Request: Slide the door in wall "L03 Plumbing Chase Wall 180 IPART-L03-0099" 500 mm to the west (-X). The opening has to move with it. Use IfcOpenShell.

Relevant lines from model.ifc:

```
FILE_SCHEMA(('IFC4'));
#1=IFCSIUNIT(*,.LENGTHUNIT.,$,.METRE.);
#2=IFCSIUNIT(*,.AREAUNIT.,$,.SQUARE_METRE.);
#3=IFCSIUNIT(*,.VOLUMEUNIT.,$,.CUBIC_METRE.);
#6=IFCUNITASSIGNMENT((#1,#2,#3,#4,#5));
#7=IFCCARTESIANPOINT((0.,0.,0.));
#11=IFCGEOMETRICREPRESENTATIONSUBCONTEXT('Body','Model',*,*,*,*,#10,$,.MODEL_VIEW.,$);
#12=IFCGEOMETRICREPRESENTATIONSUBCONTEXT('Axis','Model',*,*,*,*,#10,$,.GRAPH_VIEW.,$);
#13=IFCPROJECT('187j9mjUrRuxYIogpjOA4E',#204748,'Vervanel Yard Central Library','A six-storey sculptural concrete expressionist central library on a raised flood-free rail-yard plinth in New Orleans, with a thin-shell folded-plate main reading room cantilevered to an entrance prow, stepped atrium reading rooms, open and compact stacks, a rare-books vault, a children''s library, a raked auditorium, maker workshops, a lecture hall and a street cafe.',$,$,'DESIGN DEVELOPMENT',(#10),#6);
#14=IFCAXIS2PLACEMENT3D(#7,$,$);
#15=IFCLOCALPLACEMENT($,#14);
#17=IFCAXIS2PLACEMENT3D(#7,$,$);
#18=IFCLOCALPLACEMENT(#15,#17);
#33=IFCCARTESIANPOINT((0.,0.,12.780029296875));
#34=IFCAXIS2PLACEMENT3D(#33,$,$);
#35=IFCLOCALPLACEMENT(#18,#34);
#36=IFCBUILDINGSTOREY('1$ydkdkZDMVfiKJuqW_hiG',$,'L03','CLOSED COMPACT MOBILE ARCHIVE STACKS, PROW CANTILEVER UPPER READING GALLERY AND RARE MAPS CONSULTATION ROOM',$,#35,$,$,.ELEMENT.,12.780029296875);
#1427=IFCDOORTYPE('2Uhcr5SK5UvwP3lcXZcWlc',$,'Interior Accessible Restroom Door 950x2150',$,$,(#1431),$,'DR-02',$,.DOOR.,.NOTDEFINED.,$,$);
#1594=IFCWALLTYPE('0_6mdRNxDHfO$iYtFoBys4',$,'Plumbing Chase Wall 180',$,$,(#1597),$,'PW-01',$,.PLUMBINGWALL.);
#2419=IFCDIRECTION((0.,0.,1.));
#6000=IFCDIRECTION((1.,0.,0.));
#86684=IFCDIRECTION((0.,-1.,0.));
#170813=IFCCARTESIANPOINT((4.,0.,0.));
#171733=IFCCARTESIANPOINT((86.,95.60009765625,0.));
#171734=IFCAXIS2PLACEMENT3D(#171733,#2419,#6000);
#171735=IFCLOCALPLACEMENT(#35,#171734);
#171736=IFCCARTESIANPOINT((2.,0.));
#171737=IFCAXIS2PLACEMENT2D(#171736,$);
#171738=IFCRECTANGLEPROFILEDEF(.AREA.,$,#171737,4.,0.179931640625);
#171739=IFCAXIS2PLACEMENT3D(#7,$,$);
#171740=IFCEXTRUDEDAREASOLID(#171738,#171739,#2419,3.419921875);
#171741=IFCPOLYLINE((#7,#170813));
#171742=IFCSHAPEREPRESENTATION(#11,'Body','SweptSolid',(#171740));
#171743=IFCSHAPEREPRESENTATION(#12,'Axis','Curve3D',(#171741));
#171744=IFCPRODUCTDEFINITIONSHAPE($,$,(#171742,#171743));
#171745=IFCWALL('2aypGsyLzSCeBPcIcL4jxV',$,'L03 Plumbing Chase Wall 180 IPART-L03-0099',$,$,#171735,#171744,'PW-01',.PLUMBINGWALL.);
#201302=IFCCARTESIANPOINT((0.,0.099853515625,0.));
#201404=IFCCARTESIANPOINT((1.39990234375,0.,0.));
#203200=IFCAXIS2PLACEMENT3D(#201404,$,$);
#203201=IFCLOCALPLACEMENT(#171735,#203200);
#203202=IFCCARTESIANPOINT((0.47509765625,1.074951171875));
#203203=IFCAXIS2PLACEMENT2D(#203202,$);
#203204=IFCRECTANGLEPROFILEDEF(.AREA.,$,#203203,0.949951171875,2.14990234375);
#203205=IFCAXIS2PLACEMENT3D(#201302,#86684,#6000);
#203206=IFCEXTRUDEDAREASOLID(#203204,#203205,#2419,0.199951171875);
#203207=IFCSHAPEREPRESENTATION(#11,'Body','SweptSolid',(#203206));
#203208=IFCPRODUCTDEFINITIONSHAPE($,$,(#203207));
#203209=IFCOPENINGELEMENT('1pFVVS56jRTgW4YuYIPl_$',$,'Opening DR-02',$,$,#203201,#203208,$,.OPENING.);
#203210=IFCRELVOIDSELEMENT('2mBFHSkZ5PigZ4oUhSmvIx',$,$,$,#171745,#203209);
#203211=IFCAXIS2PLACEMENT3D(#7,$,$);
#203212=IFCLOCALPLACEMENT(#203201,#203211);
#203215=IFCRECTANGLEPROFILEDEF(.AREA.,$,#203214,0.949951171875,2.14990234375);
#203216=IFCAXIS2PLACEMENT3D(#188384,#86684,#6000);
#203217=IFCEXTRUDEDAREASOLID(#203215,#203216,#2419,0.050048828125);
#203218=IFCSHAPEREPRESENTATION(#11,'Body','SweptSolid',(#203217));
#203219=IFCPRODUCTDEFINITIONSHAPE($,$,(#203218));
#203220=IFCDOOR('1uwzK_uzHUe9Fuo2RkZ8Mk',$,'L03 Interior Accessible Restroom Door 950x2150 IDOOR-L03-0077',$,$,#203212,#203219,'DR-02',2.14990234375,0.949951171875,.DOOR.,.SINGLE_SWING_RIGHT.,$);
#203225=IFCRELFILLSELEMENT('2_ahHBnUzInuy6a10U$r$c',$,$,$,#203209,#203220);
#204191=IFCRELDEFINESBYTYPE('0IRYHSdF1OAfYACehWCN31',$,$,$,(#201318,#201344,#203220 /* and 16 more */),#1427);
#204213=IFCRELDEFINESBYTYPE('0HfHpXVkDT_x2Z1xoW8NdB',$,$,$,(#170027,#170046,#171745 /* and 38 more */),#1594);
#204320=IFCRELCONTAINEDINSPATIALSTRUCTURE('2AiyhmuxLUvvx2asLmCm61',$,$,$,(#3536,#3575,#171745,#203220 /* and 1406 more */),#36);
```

```python
import ifcopenshell
import ifcopenshell.api.geometry
import ifcopenshell.util.placement

model = ifcopenshell.open("model.ifc")

door = model.by_guid("1uwzK_uzHUe9Fuo2RkZ8Mk")
opening = door.FillsVoids[0].RelatingOpeningElement
wall = opening.VoidsElements[0].RelatingBuildingElement

wall_matrix = ifcopenshell.util.placement.get_local_placement(wall.ObjectPlacement)
shift = wall_matrix[:3, 0] * -0.5
before = ifcopenshell.util.placement.get_local_placement(door.ObjectPlacement)[:3, 3].copy()

# The door is placed relative to its opening, so it follows when the opening moves.
matrix = ifcopenshell.util.placement.get_local_placement(opening.ObjectPlacement)
matrix[:3, 3] += shift
ifcopenshell.api.geometry.edit_object_placement(
    model, product=opening, matrix=matrix, is_si=False, should_transform_children=True
)

after = ifcopenshell.util.placement.get_local_placement(door.ObjectPlacement)[:3, 3]
print("door moved by", (after - before).round(3) + 0.0)

model.write("model_rev.ifc")
```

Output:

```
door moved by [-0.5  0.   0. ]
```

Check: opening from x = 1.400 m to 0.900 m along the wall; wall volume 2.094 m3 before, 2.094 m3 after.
